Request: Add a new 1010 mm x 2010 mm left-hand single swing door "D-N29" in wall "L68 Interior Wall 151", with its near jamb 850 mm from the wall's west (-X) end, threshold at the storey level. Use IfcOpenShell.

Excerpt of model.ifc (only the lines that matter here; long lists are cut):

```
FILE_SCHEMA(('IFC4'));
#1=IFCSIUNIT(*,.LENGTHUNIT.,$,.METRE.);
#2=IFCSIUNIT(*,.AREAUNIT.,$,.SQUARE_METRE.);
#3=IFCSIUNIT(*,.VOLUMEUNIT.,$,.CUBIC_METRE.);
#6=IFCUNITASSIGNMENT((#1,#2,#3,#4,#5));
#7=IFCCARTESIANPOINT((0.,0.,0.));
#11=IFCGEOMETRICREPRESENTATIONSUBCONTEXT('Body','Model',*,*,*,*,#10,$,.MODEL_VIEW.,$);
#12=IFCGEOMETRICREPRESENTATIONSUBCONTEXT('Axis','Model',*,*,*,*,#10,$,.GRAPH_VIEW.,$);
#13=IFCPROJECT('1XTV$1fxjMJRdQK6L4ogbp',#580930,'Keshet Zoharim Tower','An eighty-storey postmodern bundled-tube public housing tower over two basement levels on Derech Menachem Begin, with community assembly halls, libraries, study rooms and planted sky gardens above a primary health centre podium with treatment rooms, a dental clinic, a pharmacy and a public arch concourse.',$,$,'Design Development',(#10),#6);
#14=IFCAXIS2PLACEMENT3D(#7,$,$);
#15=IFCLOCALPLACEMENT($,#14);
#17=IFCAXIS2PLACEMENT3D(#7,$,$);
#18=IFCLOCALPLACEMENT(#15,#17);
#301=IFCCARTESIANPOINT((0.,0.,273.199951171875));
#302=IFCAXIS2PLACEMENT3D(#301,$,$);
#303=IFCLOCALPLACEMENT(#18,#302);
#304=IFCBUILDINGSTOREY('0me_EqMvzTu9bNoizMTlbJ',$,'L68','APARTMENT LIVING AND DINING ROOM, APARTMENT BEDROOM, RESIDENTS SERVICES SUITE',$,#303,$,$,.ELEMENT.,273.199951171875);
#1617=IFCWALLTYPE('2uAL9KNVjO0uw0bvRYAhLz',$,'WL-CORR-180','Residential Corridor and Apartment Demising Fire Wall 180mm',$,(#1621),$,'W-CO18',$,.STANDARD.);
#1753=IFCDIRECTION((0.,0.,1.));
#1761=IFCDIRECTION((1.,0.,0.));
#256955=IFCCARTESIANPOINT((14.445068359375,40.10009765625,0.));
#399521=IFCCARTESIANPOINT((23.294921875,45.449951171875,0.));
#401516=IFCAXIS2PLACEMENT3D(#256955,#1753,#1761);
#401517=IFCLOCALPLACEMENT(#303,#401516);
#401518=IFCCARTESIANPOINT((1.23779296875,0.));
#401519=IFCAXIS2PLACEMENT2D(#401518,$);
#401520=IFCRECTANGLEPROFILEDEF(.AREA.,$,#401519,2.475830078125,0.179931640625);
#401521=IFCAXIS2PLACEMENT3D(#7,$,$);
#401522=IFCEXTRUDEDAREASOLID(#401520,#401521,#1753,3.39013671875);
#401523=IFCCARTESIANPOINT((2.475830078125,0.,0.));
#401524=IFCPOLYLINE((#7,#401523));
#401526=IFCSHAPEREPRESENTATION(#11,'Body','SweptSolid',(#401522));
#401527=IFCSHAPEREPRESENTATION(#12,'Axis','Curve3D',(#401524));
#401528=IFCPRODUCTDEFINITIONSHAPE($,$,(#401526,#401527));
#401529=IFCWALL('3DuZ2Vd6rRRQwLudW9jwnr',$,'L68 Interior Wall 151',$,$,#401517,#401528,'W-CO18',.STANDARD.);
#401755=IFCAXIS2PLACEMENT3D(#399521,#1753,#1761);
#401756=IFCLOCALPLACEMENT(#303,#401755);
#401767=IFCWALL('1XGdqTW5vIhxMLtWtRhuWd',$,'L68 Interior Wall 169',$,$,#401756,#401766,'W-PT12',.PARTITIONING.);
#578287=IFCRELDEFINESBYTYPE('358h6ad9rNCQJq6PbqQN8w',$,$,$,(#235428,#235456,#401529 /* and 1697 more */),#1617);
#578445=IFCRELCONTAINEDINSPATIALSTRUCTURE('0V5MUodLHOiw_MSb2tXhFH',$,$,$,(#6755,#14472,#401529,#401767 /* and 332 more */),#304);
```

```python
import numpy as np
import ifcopenshell
import ifcopenshell.api.feature
import ifcopenshell.api.geometry
import ifcopenshell.api.root
import ifcopenshell.api.spatial
import ifcopenshell.geom
import ifcopenshell.util.element
import ifcopenshell.util.placement
import ifcopenshell.util.representation
import ifcopenshell.util.shape
import ifcopenshell.util.unit

model = ifcopenshell.open("model.ifc")
unit_scale = ifcopenshell.util.unit.calculate_unit_scale(model)
settings = ifcopenshell.geom.settings()


def volume(element):
    """Net volume in cubic metres, openings subtracted."""
    shape = ifcopenshell.geom.create_shape(settings, element)
    return ifcopenshell.util.shape.get_volume(shape.geometry)


wall = model.by_guid("3DuZ2Vd6rRRQwLudW9jwnr")
storey = ifcopenshell.util.element.get_container(wall, ifc_class="IfcBuildingStorey")
context = ifcopenshell.util.representation.get_context(model, "Model", "Body", "MODEL_VIEW")
before = volume(wall)

width, height, from_end, sill = 1.01, 2.01, 0.85, 0.0  # metres

# The wall runs along its own X axis, and the end named is its -X end.
wall_shape = ifcopenshell.geom.create_shape(settings, wall)
x, y, z = ifcopenshell.util.shape.get_vertices(wall_shape.geometry).T
start = x.min() + from_end
face, thickness = float(y.min()), float(y.max() - y.min())
wall_matrix = ifcopenshell.util.placement.get_local_placement(wall.ObjectPlacement)
level = ifcopenshell.util.placement.get_local_placement(storey.ObjectPlacement)[2, 3]


def in_wall(x, y):
    """Placement at x, y metres in the wall's axes, at sill height."""
    matrix = wall_matrix.copy()
    matrix[:, 3] = wall_matrix @ np.array([x / unit_scale, y / unit_scale, 0.0, 1.0])
    matrix[2, 3] = level + sill / unit_scale
    return matrix


# Opening: a box that overshoots both wall faces by 50 mm.
opening = ifcopenshell.api.root.create_entity(model, ifc_class="IfcOpeningElement", predefined_type="OPENING")
box = ifcopenshell.api.geometry.add_wall_representation(
    model, context=context, length=width, height=height, thickness=thickness + 0.1
)
ifcopenshell.api.geometry.assign_representation(model, product=opening, representation=box)
ifcopenshell.api.geometry.edit_object_placement(model, product=opening, matrix=in_wall(start, face - 0.05), is_si=False)
ifcopenshell.api.feature.add_feature(model, feature=opening, element=wall)

door = ifcopenshell.api.root.create_entity(model, ifc_class="IfcDoor", name="D-N29", predefined_type="DOOR")
door.OverallWidth, door.OverallHeight = width / unit_scale, height / unit_scale
door.OperationType = "SINGLE_SWING_LEFT"
body = ifcopenshell.api.geometry.add_door_representation(
    model,
    context=context,
    overall_width=door.OverallWidth,
    overall_height=door.OverallHeight,
    operation_type="SINGLE_SWING_LEFT",
    lining_properties={"LiningDepth": thickness / unit_scale, "ThresholdDepth": thickness / unit_scale},
)
ifcopenshell.api.geometry.assign_representation(model, product=door, representation=body)
ifcopenshell.api.spatial.assign_container(model, products=[door], relating_structure=storey)
ifcopenshell.api.feature.add_filling(model, opening=opening, element=door)

# The lining spans the wall, so the door starts at the wall face.
ifcopenshell.api.geometry.edit_object_placement(model, product=door, matrix=in_wall(start, face), is_si=False)

after = volume(wall)

print(f"wall volume {before:.3f} -> {after:.3f} m3")

model.write("model_edited.ifc")
```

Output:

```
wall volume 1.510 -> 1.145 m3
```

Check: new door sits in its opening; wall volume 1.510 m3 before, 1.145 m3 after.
